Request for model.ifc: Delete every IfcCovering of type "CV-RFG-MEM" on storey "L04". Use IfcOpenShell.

First a look at what the model holds.

```python
import ifcopenshell
import ifcopenshell.util.element

model = ifcopenshell.open("model.ifc")
print(model.schema)
storey = next(s for s in model.by_type("IfcBuildingStorey") if s.Name == "L04")
coverings = [e for e in ifcopenshell.util.element.get_decomposition(storey) if e.is_a("IfcCovering")]
seen = {}
for e in coverings:
    element_type = ifcopenshell.util.element.get_type(e)
    name = element_type.Name if element_type not in (None, e) else None
    seen[name] = seen.get(name, 0) + 1
for name, count in sorted(seen.items(), key=str):
    print(count, "x", name)
```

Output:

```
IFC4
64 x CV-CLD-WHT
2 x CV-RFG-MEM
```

```python
import ifcopenshell
import ifcopenshell.api.root
import ifcopenshell.util.element

model = ifcopenshell.open("model.ifc")

storey = next(s for s in model.by_type("IfcBuildingStorey") if s.Name == "L04")
coverings = [e for e in ifcopenshell.util.element.get_decomposition(storey) if e.is_a("IfcCovering")]
targets = [e for e in coverings if (t := ifcopenshell.util.element.get_type(e)) not in (None, e) and t.Name == "CV-RFG-MEM"]

for e in targets:
    ifcopenshell.api.root.remove_product(model, product=e)
print(len(targets), "removed")

model.write("model-out.ifc")
```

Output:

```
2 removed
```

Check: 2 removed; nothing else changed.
